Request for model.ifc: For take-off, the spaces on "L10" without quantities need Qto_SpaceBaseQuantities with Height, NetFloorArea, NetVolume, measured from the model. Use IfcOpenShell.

First a look at what the model holds.

```python
import ifcopenshell
import ifcopenshell.util.element
import ifcopenshell.util.unit

model = ifcopenshell.open("model.ifc")
print(model.schema)
for unit_type in ("LENGTHUNIT", "AREAUNIT", "VOLUMEUNIT"):
    print(unit_type, ifcopenshell.util.unit.calculate_unit_scale(model, unit_type))
storey = next(s for s in model.by_type("IfcBuildingStorey") if s.Name == "L10")
spaces = [e for e in ifcopenshell.util.element.get_decomposition(storey) if e.is_a("IfcSpace")]
for e in sorted(spaces, key=lambda e: e.id()):
    print(e.id(), e.is_a(), e.Name, list(ifcopenshell.util.element.get_psets(e, qtos_only=True)), sep=" | ")
```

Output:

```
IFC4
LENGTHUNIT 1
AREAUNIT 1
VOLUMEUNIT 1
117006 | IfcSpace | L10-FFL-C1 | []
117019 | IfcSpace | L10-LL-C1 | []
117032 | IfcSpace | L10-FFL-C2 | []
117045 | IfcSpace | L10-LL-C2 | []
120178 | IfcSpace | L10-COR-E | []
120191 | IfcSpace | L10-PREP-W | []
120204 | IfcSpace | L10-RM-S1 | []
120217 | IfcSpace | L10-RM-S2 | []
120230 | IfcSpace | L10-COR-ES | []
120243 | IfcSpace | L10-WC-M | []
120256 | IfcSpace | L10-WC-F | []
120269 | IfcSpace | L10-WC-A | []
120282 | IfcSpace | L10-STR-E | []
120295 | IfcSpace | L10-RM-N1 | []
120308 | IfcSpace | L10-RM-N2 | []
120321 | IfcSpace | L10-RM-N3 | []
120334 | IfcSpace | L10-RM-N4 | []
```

```python
import ifcopenshell
import ifcopenshell.api.pset
import ifcopenshell.geom
import ifcopenshell.util.element
import ifcopenshell.util.shape
import ifcopenshell.util.unit

model = ifcopenshell.open("model.ifc")
unit_scale = ifcopenshell.util.unit.calculate_unit_scale(model)
area_scale = ifcopenshell.util.unit.calculate_unit_scale(model, "AREAUNIT")
volume_scale = ifcopenshell.util.unit.calculate_unit_scale(model, "VOLUMEUNIT")
settings = ifcopenshell.geom.settings()

storey = next(s for s in model.by_type("IfcBuildingStorey") if s.Name == "L10")
spaces = [e for e in ifcopenshell.util.element.get_decomposition(storey) if e.is_a("IfcSpace")]

for e in sorted(spaces, key=lambda e: e.id()):
    if ifcopenshell.util.element.get_psets(e, qtos_only=True, should_inherit=False):
        continue
    # Geometry comes back in metres, in the element's own axes.
    shape = ifcopenshell.geom.create_shape(settings, e)
    values = {
        "Height": ifcopenshell.util.shape.get_z(shape.geometry) / unit_scale,
        "NetFloorArea": ifcopenshell.util.shape.get_footprint_area(shape.geometry) / area_scale,
        "NetVolume": ifcopenshell.util.shape.get_volume(shape.geometry) / volume_scale,
    }
    qto = ifcopenshell.api.pset.add_qto(model, product=e, name="Qto_SpaceBaseQuantities")
    ifcopenshell.api.pset.edit_qto(model, qto=qto, properties=values)
    print(e.id(), {k: round(v, 3) for k, v in values.items()})

model.write("model_rev.ifc")
```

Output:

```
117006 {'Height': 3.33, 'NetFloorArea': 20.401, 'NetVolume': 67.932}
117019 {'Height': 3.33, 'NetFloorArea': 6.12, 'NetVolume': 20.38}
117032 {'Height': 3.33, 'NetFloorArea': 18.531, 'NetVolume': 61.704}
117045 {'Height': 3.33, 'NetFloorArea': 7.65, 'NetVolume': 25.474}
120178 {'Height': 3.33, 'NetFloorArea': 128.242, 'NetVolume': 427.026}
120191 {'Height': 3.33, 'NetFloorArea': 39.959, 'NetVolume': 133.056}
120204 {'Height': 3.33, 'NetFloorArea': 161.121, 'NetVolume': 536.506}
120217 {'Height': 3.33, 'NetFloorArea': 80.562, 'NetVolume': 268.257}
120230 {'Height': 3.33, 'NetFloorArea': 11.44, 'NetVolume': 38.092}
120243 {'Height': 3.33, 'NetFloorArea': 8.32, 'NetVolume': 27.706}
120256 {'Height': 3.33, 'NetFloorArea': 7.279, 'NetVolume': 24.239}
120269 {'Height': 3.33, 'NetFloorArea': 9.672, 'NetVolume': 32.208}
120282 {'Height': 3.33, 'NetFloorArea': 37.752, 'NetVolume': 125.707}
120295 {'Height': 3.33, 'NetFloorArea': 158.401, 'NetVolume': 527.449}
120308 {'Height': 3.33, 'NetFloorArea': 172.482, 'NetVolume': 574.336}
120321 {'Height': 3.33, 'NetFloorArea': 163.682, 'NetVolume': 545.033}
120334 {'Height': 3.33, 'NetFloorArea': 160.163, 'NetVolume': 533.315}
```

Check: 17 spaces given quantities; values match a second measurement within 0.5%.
